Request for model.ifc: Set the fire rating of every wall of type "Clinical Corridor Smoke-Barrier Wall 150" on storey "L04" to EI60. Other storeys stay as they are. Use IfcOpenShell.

First a look at what the model holds.

```python
import ifcopenshell
import ifcopenshell.util.element

model = ifcopenshell.open("model.ifc")
print(model.schema)
storey = next(s for s in model.by_type("IfcBuildingStorey") if s.Name == "L04")
walls = [e for e in ifcopenshell.util.element.get_decomposition(storey) if e.is_a("IfcWall")]
seen = {}
for e in walls:
    element_type = ifcopenshell.util.element.get_type(e)
    key = (element_type.Name if element_type != e and element_type else None, ifcopenshell.util.element.get_pset(e, "Pset_WallCommon", "FireRating"))
    seen[key] = seen.get(key, 0) + 1
for (name, value), count in sorted(seen.items(), key=str):
    print(count, "x", name, "|", value)
```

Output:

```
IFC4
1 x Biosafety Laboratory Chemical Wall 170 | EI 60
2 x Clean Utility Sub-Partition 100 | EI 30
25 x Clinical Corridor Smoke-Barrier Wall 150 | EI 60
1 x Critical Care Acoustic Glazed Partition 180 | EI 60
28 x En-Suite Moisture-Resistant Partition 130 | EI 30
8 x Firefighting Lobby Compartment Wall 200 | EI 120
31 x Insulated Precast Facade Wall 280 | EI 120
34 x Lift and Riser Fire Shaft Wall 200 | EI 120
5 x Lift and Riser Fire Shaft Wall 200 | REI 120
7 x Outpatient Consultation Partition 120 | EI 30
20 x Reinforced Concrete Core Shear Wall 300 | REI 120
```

```python
import ifcopenshell
import ifcopenshell.api.pset
import ifcopenshell.util.element

model = ifcopenshell.open("model.ifc")

storey = next(s for s in model.by_type("IfcBuildingStorey") if s.Name == "L04")
walls = [e for e in ifcopenshell.util.element.get_decomposition(storey) if e.is_a("IfcWall")]

count = 0
for e in walls:
    element_type = ifcopenshell.util.element.get_type(e)
    if element_type in (None, e) or element_type.Name != "Clinical Corridor Smoke-Barrier Wall 150":
        continue
    # add_pset returns the element's existing set when there is one.
    pset = ifcopenshell.api.pset.add_pset(model, product=e, name="Pset_WallCommon")
    ifcopenshell.api.pset.edit_pset(model, pset=pset, properties={"FireRating": "EI60"})
    count += 1

print(count, "walls updated")

model.write("model_rev.ifc")
```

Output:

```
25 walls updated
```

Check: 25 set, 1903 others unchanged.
